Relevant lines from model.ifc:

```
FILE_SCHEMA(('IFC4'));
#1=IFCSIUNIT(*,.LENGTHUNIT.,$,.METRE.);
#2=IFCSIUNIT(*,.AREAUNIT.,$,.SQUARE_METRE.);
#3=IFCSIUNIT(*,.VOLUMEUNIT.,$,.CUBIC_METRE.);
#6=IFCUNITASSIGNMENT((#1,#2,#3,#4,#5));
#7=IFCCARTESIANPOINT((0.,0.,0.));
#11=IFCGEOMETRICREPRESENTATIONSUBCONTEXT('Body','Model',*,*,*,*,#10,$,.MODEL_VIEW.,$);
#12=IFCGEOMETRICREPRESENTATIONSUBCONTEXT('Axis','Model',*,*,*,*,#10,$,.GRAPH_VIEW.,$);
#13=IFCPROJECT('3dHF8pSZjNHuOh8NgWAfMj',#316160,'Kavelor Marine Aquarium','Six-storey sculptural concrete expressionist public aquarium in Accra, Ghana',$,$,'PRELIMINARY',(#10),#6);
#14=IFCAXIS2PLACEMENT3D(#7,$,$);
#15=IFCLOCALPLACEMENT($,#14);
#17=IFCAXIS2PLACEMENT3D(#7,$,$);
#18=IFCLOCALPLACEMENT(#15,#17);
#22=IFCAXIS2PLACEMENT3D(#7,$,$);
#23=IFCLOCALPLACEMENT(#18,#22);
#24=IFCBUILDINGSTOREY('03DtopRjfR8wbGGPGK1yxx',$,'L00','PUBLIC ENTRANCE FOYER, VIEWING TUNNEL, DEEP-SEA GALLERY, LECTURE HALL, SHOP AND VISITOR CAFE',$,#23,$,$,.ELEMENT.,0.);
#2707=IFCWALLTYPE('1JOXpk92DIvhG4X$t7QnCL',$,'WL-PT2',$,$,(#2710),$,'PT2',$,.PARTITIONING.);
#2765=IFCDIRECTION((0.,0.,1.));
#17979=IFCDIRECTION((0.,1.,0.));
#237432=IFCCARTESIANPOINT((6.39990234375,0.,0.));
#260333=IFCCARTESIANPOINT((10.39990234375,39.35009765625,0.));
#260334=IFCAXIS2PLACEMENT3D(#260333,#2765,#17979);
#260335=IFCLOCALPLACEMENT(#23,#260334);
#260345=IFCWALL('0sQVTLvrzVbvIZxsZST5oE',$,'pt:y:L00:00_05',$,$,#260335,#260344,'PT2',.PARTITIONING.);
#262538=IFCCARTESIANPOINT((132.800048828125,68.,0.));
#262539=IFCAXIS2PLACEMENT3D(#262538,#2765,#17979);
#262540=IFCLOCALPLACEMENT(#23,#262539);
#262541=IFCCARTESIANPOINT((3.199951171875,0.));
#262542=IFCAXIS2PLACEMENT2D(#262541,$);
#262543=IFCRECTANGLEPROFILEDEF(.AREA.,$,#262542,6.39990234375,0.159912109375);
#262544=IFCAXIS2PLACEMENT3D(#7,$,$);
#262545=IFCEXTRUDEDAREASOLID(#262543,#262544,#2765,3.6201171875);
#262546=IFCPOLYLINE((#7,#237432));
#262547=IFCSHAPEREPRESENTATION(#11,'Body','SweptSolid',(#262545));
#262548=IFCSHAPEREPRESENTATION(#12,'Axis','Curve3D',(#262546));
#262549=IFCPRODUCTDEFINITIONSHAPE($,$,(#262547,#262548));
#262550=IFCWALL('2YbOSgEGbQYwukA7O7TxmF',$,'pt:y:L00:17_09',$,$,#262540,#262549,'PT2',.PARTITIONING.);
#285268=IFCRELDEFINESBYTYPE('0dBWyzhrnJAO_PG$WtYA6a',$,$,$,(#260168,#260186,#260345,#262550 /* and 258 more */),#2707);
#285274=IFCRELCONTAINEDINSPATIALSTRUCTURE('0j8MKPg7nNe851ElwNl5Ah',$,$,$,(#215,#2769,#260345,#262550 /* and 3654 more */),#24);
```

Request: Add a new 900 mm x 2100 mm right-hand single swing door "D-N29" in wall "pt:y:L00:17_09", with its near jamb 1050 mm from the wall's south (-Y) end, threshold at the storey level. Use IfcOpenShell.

```python
import numpy as np
import ifcopenshell
import ifcopenshell.api.feature
import ifcopenshell.api.geometry
import ifcopenshell.api.root
import ifcopenshell.api.spatial
import ifcopenshell.geom
import ifcopenshell.util.element
import ifcopenshell.util.placement
import ifcopenshell.util.representation
import ifcopenshell.util.shape
import ifcopenshell.util.unit

model = ifcopenshell.open("model.ifc")
unit_scale = ifcopenshell.util.unit.calculate_unit_scale(model)
settings = ifcopenshell.geom.settings()


def volume(element):
    """Net volume in cubic metres, openings subtracted."""
    shape = ifcopenshell.geom.create_shape(settings, element)
    return ifcopenshell.util.shape.get_volume(shape.geometry)


wall = model.by_id(262550)
storey = ifcopenshell.util.element.get_container(wall, ifc_class="IfcBuildingStorey")
context = ifcopenshell.util.representation.get_context(model, "Model", "Body", "MODEL_VIEW")
before = volume(wall)

width, height, from_end, sill = 0.9, 2.1, 1.05, 0.0  # metres

# The wall runs along its own X axis, and the end named is its -X end.
wall_shape = ifcopenshell.geom.create_shape(settings, wall)
x, y, z = ifcopenshell.util.shape.get_vertices(wall_shape.geometry).T
start = x.min() + from_end
face, thickness = float(y.min()), float(y.max() - y.min())
wall_matrix = ifcopenshell.util.placement.get_local_placement(wall.ObjectPlacement)
level = ifcopenshell.util.placement.get_local_placement(storey.ObjectPlacement)[2, 3]


def in_wall(x, y):
    """Placement at x, y metres in the wall's axes, at sill height."""
    matrix = wall_matrix.copy()
    matrix[:, 3] = wall_matrix @ np.array([x / unit_scale, y / unit_scale, 0.0, 1.0])
    matrix[2, 3] = level + sill / unit_scale
    return matrix


# Opening: a box that overshoots both wall faces by 50 mm.
opening = ifcopenshell.api.root.create_entity(model, ifc_class="IfcOpeningElement", predefined_type="OPENING")
box = ifcopenshell.api.geometry.add_wall_representation(
    model, context=context, length=width, height=height, thickness=thickness + 0.1
)
ifcopenshell.api.geometry.assign_representation(model, product=opening, representation=box)
ifcopenshell.api.geometry.edit_object_placement(model, product=opening, matrix=in_wall(start, face - 0.05), is_si=False)
ifcopenshell.api.feature.add_feature(model, feature=opening, element=wall)

door = ifcopenshell.api.root.create_entity(model, ifc_class="IfcDoor", name="D-N29", predefined_type="DOOR")
door.OverallWidth, door.OverallHeight = width / unit_scale, height / unit_scale
door.OperationType = "SINGLE_SWING_RIGHT"
body = ifcopenshell.api.geometry.add_door_representation(
    model,
    context=context,
    overall_width=door.OverallWidth,
    overall_height=door.OverallHeight,
    operation_type="SINGLE_SWING_RIGHT",
    lining_properties={"LiningDepth": thickness / unit_scale, "ThresholdDepth": thickness / unit_scale},
)
ifcopenshell.api.geometry.assign_representation(model, product=door, representation=body)
ifcopenshell.api.spatial.assign_container(model, products=[door], relating_structure=storey)
ifcopenshell.api.feature.add_filling(model, opening=opening, element=door)

# The lining spans the wall, so the door starts at the wall face.
ifcopenshell.api.geometry.edit_object_placement(model, product=door, matrix=in_wall(start, face), is_si=False)

after = volume(wall)

print(f"wall volume {before:.3f} -> {after:.3f} m3")

model.write("model_edited.ifc")
```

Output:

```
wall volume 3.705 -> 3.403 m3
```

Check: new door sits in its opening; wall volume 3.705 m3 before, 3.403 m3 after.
